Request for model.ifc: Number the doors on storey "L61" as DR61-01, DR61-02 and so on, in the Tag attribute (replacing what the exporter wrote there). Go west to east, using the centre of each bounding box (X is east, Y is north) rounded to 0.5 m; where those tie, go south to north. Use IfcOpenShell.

First a look at what the model holds.

```python
import ifcopenshell
import ifcopenshell.util.element
import ifcopenshell.util.placement

model = ifcopenshell.open("model.ifc")
print(model.schema)
storey = next(s for s in model.by_type("IfcBuildingStorey") if s.Name == "L61")
doors = [e for e in ifcopenshell.util.element.get_decomposition(storey) if e.is_a("IfcDoor")]
for e in sorted(doors, key=lambda e: e.id()):
    origin = ifcopenshell.util.placement.get_local_placement(e.ObjectPlacement)[:3, 3]
    print(e.id(), e.Tag, e.Name, origin.round(2) + 0.0, sep=" | ")
```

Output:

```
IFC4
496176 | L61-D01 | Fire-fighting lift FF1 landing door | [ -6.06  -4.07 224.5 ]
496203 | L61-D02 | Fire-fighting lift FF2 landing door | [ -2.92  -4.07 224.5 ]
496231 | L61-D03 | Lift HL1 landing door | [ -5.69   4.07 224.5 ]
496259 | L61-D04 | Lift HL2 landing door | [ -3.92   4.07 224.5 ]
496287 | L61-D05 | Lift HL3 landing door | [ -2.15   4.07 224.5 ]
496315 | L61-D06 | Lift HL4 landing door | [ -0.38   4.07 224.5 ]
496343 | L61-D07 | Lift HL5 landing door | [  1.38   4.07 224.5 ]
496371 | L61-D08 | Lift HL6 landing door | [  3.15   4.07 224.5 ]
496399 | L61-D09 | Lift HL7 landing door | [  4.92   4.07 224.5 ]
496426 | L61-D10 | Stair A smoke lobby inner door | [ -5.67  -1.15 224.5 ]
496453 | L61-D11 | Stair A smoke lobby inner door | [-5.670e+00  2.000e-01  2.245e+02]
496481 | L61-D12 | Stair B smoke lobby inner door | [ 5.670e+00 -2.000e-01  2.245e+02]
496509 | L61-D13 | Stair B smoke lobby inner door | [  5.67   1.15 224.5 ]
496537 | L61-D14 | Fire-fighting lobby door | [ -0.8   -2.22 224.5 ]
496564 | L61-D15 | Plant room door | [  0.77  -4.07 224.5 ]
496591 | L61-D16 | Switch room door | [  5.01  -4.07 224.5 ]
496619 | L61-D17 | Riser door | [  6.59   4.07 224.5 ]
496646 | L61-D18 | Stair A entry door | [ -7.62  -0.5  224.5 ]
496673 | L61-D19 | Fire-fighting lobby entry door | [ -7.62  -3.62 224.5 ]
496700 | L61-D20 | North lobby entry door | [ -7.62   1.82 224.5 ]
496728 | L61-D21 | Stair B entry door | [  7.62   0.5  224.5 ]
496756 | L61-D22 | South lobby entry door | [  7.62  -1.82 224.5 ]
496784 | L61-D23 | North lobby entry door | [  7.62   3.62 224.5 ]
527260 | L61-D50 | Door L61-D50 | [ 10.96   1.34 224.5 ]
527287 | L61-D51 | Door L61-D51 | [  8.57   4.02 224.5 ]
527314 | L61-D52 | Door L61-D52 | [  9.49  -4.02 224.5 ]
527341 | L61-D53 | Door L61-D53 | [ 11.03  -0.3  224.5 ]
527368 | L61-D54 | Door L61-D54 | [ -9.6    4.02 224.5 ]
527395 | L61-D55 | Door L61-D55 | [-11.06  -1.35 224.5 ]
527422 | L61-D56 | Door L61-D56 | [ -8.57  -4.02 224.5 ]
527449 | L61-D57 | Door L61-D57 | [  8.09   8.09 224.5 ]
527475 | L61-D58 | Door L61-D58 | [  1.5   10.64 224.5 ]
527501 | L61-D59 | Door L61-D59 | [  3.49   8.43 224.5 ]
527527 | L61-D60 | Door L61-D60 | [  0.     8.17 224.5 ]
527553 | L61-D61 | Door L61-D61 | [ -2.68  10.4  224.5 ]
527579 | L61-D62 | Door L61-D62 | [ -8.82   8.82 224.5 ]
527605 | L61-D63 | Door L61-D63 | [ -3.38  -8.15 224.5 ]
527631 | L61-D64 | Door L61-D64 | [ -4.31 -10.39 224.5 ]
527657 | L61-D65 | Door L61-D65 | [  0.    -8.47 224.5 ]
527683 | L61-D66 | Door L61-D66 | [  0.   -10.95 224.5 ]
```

```python
import ifcopenshell
import ifcopenshell.geom
import ifcopenshell.util.element
import ifcopenshell.util.shape

model = ifcopenshell.open("model.ifc")
settings = ifcopenshell.geom.settings()
settings.set("use-world-coords", True)


def centre(element):
    shape = ifcopenshell.geom.create_shape(settings, element)
    return ifcopenshell.util.shape.get_bbox_centroid(shape.geometry)


storey = next(s for s in model.by_type("IfcBuildingStorey") if s.Name == "L61")
doors = [e for e in ifcopenshell.util.element.get_decomposition(storey) if e.is_a("IfcDoor")]

# Insertion points can sit at a corner or the storey origin, so sort by the geometry (in metres).
centres = {e: centre(e) for e in doors}
doors.sort(key=lambda e: (round(centres[e][0] / 0.5), centres[e][1]))

for i, e in enumerate(doors, start=1):
    number = f"DR61-{i:02d}"
    e.Tag = number
    print(e.id(), number)

model.write("model-out.ifc")
```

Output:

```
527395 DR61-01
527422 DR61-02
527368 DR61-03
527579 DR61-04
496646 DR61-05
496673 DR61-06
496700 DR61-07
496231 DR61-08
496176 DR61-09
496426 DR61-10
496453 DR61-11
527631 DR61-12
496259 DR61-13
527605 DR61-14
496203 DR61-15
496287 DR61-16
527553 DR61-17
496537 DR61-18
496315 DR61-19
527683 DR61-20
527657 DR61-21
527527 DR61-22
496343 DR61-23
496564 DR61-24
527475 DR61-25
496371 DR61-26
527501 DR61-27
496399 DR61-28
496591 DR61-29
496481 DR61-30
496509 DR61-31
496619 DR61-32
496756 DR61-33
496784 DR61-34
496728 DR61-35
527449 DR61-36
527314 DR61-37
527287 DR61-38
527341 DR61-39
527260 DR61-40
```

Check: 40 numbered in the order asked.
